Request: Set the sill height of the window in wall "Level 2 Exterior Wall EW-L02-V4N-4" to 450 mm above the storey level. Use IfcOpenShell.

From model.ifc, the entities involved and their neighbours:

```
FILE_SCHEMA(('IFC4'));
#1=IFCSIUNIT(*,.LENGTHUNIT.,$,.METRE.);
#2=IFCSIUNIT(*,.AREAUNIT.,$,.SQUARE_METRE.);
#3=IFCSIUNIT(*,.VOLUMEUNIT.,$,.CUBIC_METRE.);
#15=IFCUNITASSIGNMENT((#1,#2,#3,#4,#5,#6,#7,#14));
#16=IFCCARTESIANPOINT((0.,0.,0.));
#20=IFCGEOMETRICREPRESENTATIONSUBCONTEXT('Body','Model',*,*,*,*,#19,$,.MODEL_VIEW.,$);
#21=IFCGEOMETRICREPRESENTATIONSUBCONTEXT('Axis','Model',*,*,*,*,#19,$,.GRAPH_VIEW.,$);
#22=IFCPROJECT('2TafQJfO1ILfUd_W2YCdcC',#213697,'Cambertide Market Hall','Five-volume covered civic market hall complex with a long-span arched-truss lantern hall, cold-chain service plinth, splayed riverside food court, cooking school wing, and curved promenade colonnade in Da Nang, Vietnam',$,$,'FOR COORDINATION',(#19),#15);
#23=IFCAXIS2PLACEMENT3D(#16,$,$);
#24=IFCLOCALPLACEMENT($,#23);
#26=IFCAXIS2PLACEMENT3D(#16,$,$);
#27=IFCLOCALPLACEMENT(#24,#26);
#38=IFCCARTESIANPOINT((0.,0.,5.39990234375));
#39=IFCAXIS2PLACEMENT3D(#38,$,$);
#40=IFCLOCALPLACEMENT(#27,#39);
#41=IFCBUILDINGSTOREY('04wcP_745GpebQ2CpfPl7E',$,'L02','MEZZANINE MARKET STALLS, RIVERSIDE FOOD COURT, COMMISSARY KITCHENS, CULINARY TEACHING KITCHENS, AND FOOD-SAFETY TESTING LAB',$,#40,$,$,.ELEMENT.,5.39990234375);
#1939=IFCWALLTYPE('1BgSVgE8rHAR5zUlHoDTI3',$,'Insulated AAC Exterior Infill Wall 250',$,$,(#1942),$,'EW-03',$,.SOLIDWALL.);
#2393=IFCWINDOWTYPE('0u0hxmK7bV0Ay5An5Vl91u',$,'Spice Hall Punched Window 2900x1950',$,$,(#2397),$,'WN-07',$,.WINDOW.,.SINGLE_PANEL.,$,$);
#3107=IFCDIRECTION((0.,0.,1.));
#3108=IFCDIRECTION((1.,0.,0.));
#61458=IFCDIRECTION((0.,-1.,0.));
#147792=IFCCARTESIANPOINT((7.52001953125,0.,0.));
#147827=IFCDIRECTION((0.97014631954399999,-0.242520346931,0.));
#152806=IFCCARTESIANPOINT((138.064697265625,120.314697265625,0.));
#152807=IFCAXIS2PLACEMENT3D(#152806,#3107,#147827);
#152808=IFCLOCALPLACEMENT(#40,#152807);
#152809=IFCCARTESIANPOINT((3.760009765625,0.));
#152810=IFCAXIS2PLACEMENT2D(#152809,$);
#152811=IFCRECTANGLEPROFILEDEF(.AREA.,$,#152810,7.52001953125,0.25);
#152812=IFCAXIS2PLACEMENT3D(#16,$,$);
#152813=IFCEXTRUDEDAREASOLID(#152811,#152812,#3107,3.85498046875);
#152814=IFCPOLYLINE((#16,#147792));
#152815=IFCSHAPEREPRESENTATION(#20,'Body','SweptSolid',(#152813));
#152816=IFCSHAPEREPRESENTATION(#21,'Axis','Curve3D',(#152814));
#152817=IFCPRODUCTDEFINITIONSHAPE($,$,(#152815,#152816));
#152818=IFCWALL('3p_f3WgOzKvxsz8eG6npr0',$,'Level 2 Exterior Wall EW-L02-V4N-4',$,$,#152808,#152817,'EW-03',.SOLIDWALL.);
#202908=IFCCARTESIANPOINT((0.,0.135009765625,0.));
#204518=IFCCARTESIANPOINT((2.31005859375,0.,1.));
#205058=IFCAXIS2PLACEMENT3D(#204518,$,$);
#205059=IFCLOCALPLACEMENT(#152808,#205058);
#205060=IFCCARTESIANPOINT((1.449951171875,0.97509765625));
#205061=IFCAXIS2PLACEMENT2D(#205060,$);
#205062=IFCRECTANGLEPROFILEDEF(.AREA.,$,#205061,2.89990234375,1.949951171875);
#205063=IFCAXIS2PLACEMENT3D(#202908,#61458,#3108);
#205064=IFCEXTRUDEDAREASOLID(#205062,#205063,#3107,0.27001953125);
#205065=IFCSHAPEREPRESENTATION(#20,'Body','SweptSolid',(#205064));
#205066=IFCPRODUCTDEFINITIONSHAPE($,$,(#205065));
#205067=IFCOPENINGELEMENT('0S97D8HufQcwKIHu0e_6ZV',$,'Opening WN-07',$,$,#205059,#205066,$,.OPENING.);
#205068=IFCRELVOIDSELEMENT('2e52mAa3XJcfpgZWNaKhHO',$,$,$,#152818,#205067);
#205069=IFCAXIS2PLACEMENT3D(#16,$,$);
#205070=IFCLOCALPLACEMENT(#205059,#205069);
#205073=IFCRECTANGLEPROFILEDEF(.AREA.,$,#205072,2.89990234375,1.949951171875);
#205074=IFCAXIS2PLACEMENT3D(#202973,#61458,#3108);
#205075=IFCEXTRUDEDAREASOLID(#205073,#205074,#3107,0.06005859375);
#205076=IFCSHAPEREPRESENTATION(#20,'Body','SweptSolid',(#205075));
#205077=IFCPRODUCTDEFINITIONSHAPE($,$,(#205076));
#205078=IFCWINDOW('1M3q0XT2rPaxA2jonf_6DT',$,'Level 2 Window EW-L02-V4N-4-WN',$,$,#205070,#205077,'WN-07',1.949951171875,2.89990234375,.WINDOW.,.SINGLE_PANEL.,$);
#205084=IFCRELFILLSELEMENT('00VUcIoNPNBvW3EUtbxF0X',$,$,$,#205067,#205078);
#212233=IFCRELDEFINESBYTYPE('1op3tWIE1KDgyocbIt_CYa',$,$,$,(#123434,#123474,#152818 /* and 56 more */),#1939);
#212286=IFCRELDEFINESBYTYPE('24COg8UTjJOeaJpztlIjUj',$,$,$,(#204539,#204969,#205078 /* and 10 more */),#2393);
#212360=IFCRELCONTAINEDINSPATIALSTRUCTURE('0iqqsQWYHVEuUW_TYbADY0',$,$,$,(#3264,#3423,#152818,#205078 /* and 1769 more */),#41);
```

```python
import numpy as np
import ifcopenshell
import ifcopenshell.api.geometry
import ifcopenshell.geom
import ifcopenshell.util.element
import ifcopenshell.util.placement
import ifcopenshell.util.shape
import ifcopenshell.util.unit

model = ifcopenshell.open("model.ifc")
unit_scale = ifcopenshell.util.unit.calculate_unit_scale(model)

window = model.by_guid("1M3q0XT2rPaxA2jonf_6DT")
opening = window.FillsVoids[0].RelatingOpeningElement
storey = ifcopenshell.util.element.get_container(window, ifc_class="IfcBuildingStorey")
level = ifcopenshell.util.placement.get_local_placement(storey.ObjectPlacement)[2, 3]

# The opening's origin need not be at the sill, so measure its lowest point.
shape = ifcopenshell.geom.create_shape(ifcopenshell.geom.settings(), opening)
bottom = ifcopenshell.util.shape.get_shape_bottom_elevation(shape, shape.geometry) / unit_scale
dz = level + 0.45 / unit_scale - bottom

shift = np.array([0.0, 0.0, dz])
# The window is placed relative to its opening, so it follows when the opening moves.
matrix = ifcopenshell.util.placement.get_local_placement(opening.ObjectPlacement)
matrix[:3, 3] += shift
ifcopenshell.api.geometry.edit_object_placement(
    model, product=opening, matrix=matrix, is_si=False, should_transform_children=True
)

print(f"moved by {dz * unit_scale:+.3f} m")

model.write("model_v2.ifc")
```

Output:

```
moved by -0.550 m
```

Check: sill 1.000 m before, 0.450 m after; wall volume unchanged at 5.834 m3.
